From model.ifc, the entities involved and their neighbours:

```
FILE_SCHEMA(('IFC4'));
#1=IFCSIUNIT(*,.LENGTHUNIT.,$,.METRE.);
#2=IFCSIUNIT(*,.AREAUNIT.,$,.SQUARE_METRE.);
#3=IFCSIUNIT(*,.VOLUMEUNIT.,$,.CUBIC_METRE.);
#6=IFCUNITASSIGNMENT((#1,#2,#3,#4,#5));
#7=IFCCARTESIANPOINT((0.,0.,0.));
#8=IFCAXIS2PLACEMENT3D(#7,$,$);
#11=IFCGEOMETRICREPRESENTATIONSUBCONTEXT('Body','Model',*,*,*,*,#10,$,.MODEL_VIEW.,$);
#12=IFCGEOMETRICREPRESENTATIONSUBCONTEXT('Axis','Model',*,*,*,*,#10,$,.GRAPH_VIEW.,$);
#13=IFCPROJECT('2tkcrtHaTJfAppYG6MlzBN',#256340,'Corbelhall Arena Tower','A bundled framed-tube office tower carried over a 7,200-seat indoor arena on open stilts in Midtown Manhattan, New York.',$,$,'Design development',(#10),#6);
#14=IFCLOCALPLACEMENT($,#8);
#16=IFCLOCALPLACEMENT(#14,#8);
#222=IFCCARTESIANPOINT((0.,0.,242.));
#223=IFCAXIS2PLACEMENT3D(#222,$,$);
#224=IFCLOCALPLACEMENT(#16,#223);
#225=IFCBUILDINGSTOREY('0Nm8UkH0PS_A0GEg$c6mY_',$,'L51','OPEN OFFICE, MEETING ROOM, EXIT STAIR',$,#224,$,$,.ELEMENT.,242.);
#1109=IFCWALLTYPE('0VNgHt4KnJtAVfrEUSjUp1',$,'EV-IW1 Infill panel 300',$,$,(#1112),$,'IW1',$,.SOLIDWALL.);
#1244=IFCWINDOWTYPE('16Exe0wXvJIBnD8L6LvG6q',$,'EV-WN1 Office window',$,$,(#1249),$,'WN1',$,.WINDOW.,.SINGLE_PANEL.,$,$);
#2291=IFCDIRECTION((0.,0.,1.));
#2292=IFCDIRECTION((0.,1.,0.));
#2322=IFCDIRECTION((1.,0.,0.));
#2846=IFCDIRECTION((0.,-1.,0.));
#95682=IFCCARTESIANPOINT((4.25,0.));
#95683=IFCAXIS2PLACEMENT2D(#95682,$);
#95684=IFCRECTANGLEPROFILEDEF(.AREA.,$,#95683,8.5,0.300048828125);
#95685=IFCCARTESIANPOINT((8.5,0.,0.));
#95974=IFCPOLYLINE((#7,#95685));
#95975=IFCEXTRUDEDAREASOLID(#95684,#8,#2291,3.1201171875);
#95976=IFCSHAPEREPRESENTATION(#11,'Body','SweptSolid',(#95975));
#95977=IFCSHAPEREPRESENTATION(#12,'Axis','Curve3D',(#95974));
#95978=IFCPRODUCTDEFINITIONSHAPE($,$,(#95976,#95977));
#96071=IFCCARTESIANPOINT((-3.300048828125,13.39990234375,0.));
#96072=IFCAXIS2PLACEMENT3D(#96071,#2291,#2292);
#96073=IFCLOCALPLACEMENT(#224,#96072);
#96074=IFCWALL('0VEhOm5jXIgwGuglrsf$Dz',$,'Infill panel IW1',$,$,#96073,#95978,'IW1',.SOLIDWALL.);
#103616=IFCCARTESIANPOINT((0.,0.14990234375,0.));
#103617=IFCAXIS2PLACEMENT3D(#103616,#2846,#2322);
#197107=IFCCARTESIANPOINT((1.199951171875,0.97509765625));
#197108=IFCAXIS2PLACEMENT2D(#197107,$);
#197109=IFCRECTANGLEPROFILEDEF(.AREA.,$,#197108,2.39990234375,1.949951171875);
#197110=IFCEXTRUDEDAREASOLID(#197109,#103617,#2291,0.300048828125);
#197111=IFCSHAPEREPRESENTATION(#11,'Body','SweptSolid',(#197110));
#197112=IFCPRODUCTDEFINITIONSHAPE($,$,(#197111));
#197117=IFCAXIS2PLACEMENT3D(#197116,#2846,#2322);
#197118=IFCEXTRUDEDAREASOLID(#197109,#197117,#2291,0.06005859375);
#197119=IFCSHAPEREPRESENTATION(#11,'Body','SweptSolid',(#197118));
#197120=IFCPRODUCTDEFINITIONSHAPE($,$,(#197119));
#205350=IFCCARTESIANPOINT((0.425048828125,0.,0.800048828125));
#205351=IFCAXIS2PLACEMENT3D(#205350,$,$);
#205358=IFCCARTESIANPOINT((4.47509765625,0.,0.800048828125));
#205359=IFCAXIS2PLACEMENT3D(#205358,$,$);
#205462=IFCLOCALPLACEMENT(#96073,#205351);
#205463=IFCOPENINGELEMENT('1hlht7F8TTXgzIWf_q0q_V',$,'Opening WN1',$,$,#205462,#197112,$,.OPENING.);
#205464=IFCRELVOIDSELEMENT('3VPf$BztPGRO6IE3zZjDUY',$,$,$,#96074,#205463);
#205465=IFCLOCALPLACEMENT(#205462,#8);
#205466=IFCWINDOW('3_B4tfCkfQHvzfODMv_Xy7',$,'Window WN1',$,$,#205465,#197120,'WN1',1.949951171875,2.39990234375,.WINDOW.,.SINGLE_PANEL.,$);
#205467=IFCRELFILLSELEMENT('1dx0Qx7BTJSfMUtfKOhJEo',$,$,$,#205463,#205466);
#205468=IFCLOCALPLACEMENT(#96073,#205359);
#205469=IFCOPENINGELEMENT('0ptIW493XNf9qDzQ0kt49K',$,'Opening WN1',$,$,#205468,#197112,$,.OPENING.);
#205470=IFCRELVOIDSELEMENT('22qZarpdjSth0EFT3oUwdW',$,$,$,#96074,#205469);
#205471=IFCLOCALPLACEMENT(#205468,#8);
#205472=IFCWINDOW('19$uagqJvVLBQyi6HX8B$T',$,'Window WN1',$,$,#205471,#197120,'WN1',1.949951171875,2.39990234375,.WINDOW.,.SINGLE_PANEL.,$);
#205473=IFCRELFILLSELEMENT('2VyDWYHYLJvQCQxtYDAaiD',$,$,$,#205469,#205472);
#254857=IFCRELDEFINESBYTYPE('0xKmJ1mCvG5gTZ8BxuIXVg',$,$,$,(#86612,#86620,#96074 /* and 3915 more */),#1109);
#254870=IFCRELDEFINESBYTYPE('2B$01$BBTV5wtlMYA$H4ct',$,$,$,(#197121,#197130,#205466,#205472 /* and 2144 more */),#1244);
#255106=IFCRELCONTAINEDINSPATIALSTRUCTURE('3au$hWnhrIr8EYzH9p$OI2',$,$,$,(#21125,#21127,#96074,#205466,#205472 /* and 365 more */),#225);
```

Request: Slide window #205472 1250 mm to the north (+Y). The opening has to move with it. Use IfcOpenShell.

```python
import ifcopenshell
import ifcopenshell.api.geometry
import ifcopenshell.util.placement
import ifcopenshell.util.unit

model = ifcopenshell.open("model.ifc")
unit_scale = ifcopenshell.util.unit.calculate_unit_scale(model)

window = model.by_guid("19$uagqJvVLBQyi6HX8B$T")
opening = window.FillsVoids[0].RelatingOpeningElement
wall = opening.VoidsElements[0].RelatingBuildingElement

wall_matrix = ifcopenshell.util.placement.get_local_placement(wall.ObjectPlacement)
shift = wall_matrix[:3, 0] * 1.25 / unit_scale
before = ifcopenshell.util.placement.get_local_placement(window.ObjectPlacement)[:3, 3].copy()

# The window is placed relative to its opening, so it follows when the opening moves.
matrix = ifcopenshell.util.placement.get_local_placement(opening.ObjectPlacement)
matrix[:3, 3] += shift
ifcopenshell.api.geometry.edit_object_placement(
    model, product=opening, matrix=matrix, is_si=False, should_transform_children=True
)

after = ifcopenshell.util.placement.get_local_placement(window.ObjectPlacement)[:3, 3]
print("window moved by", (after - before).round(3) + 0.0)

model.write("model-out.ifc")
```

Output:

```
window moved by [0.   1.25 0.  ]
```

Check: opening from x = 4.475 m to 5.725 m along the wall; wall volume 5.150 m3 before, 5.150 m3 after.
